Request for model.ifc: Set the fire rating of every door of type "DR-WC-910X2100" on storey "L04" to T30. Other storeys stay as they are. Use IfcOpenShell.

First a look at what the model holds.

```python
import ifcopenshell
import ifcopenshell.util.element

model = ifcopenshell.open("model.ifc")
print(model.schema)
storey = next(s for s in model.by_type("IfcBuildingStorey") if s.Name == "L04")
doors = [e for e in ifcopenshell.util.element.get_decomposition(storey) if e.is_a("IfcDoor")]
seen = {}
for e in doors:
    element_type = ifcopenshell.util.element.get_type(e)
    key = (element_type.Name if element_type != e and element_type else None, ifcopenshell.util.element.get_pset(e, "Pset_DoorCommon", "FireRating"))
    seen[key] = seen.get(key, 0) + 1
for (name, value), count in sorted(seen.items(), key=str):
    print(count, "x", name, "|", value)
```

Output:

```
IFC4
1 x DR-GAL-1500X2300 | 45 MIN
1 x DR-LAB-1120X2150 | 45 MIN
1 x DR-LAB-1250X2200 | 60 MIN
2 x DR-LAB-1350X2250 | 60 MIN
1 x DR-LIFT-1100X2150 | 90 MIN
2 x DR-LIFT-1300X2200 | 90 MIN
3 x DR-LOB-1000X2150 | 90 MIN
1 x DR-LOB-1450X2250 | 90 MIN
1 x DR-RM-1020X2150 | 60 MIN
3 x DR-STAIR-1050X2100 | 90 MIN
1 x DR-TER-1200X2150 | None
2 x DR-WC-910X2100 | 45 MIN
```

```python
import ifcopenshell
import ifcopenshell.api.pset
import ifcopenshell.util.element

model = ifcopenshell.open("model.ifc")

storey = next(s for s in model.by_type("IfcBuildingStorey") if s.Name == "L04")
doors = [e for e in ifcopenshell.util.element.get_decomposition(storey) if e.is_a("IfcDoor")]

count = 0
for e in doors:
    element_type = ifcopenshell.util.element.get_type(e)
    if element_type in (None, e) or element_type.Name != "DR-WC-910X2100":
        continue
    # add_pset returns the element's existing set when there is one.
    pset = ifcopenshell.api.pset.add_pset(model, product=e, name="Pset_DoorCommon")
    ifcopenshell.api.pset.edit_pset(model, pset=pset, properties={"FireRating": "T30"})
    count += 1

print(count, "doors updated")

model.write("model_edited.ifc")
```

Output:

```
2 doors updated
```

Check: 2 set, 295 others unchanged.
